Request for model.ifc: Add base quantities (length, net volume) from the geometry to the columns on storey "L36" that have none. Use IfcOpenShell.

First a look at what the model holds.

```python
import ifcopenshell
import ifcopenshell.util.element
import ifcopenshell.util.unit

model = ifcopenshell.open("model.ifc")
print(model.schema)
for unit_type in ("LENGTHUNIT", "AREAUNIT", "VOLUMEUNIT"):
    print(unit_type, ifcopenshell.util.unit.calculate_unit_scale(model, unit_type))
storey = next(s for s in model.by_type("IfcBuildingStorey") if s.Name == "L36")
columns = [e for e in ifcopenshell.util.element.get_decomposition(storey) if e.is_a("IfcColumn")]
for e in sorted(columns, key=lambda e: e.id()):
    print(e.id(), e.is_a(), e.Name, list(ifcopenshell.util.element.get_psets(e, qtos_only=True)), sep=" | ")
```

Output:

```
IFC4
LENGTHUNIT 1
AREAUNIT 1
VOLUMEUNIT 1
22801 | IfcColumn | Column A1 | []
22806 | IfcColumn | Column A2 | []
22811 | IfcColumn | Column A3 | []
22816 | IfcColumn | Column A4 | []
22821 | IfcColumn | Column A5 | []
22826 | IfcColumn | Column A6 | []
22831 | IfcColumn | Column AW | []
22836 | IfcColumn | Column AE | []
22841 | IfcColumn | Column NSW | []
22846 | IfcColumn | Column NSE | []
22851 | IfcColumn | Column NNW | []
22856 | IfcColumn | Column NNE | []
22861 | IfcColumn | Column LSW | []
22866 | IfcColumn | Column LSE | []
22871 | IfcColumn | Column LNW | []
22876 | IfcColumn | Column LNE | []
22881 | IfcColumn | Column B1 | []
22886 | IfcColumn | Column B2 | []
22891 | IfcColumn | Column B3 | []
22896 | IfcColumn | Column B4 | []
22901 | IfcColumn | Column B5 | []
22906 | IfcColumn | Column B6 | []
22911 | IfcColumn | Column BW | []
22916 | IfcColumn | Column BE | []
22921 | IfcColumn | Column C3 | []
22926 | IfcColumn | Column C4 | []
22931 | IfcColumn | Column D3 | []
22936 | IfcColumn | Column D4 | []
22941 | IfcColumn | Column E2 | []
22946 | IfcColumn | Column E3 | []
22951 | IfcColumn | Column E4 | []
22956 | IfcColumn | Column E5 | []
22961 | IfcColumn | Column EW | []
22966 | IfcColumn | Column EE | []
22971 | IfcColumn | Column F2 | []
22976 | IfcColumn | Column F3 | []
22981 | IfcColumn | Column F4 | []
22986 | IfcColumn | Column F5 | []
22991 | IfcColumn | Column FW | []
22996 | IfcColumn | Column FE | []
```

```python
import ifcopenshell
import ifcopenshell.api.pset
import ifcopenshell.geom
import ifcopenshell.util.element
import ifcopenshell.util.shape
import ifcopenshell.util.unit

model = ifcopenshell.open("model.ifc")
unit_scale = ifcopenshell.util.unit.calculate_unit_scale(model)
volume_scale = ifcopenshell.util.unit.calculate_unit_scale(model, "VOLUMEUNIT")
settings = ifcopenshell.geom.settings()

storey = next(s for s in model.by_type("IfcBuildingStorey") if s.Name == "L36")
columns = [e for e in ifcopenshell.util.element.get_decomposition(storey) if e.is_a("IfcColumn")]

for e in sorted(columns, key=lambda e: e.id()):
    if ifcopenshell.util.element.get_psets(e, qtos_only=True, should_inherit=False):
        continue
    # Geometry comes back in metres, in the element's own axes.
    shape = ifcopenshell.geom.create_shape(settings, e)
    values = {
        "Length": ifcopenshell.util.shape.get_z(shape.geometry) / unit_scale,
        "NetVolume": ifcopenshell.util.shape.get_volume(shape.geometry) / volume_scale,
    }
    qto = ifcopenshell.api.pset.add_qto(model, product=e, name="Qto_ColumnBaseQuantities")
    ifcopenshell.api.pset.edit_qto(model, qto=qto, properties=values)
    print(e.id(), {k: round(v, 3) for k, v in values.items()})

model.write("model-out.ifc")
```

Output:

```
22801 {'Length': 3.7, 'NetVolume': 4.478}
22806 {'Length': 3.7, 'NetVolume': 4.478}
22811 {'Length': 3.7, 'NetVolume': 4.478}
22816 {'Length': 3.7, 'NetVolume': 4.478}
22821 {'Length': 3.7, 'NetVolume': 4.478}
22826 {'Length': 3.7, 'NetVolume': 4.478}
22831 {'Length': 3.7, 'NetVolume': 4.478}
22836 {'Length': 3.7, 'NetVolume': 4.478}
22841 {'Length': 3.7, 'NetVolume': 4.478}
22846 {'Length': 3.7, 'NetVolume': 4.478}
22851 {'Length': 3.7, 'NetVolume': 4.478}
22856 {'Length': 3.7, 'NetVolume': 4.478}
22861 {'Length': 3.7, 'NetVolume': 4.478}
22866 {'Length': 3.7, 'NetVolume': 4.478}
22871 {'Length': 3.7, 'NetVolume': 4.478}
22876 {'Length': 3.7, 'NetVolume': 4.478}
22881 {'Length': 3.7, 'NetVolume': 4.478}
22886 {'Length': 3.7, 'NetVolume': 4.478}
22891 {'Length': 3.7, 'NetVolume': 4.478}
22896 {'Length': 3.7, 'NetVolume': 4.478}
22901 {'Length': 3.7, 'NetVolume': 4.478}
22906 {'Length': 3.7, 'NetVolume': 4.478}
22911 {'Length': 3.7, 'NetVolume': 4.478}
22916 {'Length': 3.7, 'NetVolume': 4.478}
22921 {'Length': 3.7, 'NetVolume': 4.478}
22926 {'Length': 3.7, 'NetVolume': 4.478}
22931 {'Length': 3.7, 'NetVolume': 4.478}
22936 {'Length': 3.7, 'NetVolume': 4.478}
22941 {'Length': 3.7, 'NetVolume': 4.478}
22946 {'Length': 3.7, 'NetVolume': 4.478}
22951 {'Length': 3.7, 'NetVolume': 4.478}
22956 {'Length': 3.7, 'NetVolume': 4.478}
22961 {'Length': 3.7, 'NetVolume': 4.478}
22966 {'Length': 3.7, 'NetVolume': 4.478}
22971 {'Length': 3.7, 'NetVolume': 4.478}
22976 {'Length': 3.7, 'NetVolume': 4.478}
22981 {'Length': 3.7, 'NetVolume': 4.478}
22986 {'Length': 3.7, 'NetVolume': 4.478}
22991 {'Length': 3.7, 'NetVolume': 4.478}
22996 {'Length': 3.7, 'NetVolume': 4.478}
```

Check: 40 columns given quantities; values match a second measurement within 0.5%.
